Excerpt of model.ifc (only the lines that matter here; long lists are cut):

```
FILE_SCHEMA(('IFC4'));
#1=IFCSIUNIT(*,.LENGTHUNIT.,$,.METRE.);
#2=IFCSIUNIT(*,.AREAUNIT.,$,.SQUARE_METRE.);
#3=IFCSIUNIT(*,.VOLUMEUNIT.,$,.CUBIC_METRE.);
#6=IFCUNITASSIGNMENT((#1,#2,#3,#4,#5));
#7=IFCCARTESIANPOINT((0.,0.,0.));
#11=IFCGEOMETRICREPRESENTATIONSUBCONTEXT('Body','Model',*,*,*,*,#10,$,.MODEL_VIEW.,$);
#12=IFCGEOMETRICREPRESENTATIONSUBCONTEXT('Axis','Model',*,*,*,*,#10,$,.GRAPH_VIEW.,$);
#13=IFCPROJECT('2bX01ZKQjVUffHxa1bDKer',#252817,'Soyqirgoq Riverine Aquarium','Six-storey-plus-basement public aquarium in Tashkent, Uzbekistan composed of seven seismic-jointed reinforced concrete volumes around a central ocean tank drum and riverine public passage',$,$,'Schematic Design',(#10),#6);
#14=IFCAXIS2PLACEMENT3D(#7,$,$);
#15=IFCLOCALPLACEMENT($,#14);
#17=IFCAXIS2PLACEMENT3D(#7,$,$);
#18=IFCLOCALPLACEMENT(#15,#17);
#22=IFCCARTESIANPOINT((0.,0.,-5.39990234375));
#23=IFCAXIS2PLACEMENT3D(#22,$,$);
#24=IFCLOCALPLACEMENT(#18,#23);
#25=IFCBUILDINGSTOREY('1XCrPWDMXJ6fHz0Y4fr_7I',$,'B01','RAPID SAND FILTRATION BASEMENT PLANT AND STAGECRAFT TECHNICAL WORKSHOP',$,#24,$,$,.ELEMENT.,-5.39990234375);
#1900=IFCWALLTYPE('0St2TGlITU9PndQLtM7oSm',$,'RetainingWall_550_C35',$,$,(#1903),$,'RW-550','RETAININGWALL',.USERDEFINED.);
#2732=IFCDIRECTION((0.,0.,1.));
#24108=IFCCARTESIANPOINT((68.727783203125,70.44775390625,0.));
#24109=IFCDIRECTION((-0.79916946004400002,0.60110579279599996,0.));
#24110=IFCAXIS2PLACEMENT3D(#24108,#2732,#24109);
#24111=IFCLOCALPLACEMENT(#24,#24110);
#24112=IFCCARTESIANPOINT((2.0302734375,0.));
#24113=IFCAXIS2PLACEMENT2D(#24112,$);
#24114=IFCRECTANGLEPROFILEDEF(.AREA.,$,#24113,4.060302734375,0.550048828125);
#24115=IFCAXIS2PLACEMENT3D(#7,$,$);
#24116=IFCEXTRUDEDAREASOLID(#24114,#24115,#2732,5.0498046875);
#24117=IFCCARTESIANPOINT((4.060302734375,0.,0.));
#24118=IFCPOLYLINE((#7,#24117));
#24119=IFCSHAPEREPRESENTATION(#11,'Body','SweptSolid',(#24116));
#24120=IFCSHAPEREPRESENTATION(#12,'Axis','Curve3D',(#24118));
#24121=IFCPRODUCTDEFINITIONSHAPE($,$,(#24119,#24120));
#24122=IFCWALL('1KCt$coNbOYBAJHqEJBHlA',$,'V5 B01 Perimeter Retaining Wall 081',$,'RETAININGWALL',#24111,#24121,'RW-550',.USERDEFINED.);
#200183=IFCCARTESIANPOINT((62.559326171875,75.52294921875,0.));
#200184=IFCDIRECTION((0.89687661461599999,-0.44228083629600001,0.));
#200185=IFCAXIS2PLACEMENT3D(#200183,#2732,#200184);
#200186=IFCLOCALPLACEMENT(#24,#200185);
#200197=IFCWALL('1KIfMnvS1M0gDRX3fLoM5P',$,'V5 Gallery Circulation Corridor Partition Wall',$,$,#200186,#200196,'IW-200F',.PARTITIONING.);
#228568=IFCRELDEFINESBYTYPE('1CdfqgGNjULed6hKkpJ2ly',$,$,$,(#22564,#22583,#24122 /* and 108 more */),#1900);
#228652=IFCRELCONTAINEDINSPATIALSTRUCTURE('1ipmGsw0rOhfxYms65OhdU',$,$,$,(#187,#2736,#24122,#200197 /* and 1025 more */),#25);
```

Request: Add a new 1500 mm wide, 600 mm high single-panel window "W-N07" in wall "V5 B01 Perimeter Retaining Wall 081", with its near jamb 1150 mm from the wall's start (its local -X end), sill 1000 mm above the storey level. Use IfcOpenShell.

```python
import numpy as np
import ifcopenshell
import ifcopenshell.api.feature
import ifcopenshell.api.geometry
import ifcopenshell.api.root
import ifcopenshell.api.spatial
import ifcopenshell.geom
import ifcopenshell.util.element
import ifcopenshell.util.placement
import ifcopenshell.util.representation
import ifcopenshell.util.shape
import ifcopenshell.util.unit

model = ifcopenshell.open("model.ifc")
unit_scale = ifcopenshell.util.unit.calculate_unit_scale(model)
settings = ifcopenshell.geom.settings()


def volume(element):
    """Net volume in cubic metres, openings subtracted."""
    shape = ifcopenshell.geom.create_shape(settings, element)
    return ifcopenshell.util.shape.get_volume(shape.geometry)


wall = model.by_guid("1KCt$coNbOYBAJHqEJBHlA")
storey = ifcopenshell.util.element.get_container(wall, ifc_class="IfcBuildingStorey")
context = ifcopenshell.util.representation.get_context(model, "Model", "Body", "MODEL_VIEW")
before = volume(wall)

width, height, from_end, sill = 1.5, 0.6, 1.15, 1  # metres

# The wall runs along its own X axis, and the end named is its -X end.
wall_shape = ifcopenshell.geom.create_shape(settings, wall)
x, y, z = ifcopenshell.util.shape.get_vertices(wall_shape.geometry).T
start = x.min() + from_end
face, thickness = float(y.min()), float(y.max() - y.min())
wall_matrix = ifcopenshell.util.placement.get_local_placement(wall.ObjectPlacement)
level = ifcopenshell.util.placement.get_local_placement(storey.ObjectPlacement)[2, 3]


def in_wall(x, y):
    """Placement at x, y metres in the wall's axes, at sill height."""
    matrix = wall_matrix.copy()
    matrix[:, 3] = wall_matrix @ np.array([x / unit_scale, y / unit_scale, 0.0, 1.0])
    matrix[2, 3] = level + sill / unit_scale
    return matrix


# Opening: a box that overshoots both wall faces by 50 mm.
opening = ifcopenshell.api.root.create_entity(model, ifc_class="IfcOpeningElement", predefined_type="OPENING")
box = ifcopenshell.api.geometry.add_wall_representation(
    model, context=context, length=width, height=height, thickness=thickness + 0.1
)
ifcopenshell.api.geometry.assign_representation(model, product=opening, representation=box)
ifcopenshell.api.geometry.edit_object_placement(model, product=opening, matrix=in_wall(start, face - 0.05), is_si=False)
ifcopenshell.api.feature.add_feature(model, feature=opening, element=wall)

window = ifcopenshell.api.root.create_entity(model, ifc_class="IfcWindow", name="W-N07", predefined_type="WINDOW")
window.OverallWidth, window.OverallHeight = width / unit_scale, height / unit_scale
window.PartitioningType = "SINGLE_PANEL"
body = ifcopenshell.api.geometry.add_window_representation(
    model,
    context=context,
    overall_width=window.OverallWidth,
    overall_height=window.OverallHeight,
    partition_type="SINGLE_PANEL",
)
ifcopenshell.api.geometry.assign_representation(model, product=window, representation=body)
ifcopenshell.api.spatial.assign_container(model, products=[window], relating_structure=storey)
ifcopenshell.api.feature.add_filling(model, opening=opening, element=window)

# Centre the window in the wall's thickness.
ifcopenshell.api.geometry.edit_object_placement(model, product=window, matrix=in_wall(start, face), is_si=False)
window_shape = ifcopenshell.geom.create_shape(settings, window)
depth = ifcopenshell.util.shape.get_vertices(window_shape.geometry)[:, 1]
offset = face + thickness / 2 - (depth.min() + depth.max()) / 2
ifcopenshell.api.geometry.edit_object_placement(model, product=window, matrix=in_wall(start, offset), is_si=False)

after = volume(wall)

print(f"wall volume {before:.3f} -> {after:.3f} m3")

model.write("model_updated.ifc")
```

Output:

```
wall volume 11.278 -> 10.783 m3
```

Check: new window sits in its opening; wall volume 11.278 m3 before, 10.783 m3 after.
